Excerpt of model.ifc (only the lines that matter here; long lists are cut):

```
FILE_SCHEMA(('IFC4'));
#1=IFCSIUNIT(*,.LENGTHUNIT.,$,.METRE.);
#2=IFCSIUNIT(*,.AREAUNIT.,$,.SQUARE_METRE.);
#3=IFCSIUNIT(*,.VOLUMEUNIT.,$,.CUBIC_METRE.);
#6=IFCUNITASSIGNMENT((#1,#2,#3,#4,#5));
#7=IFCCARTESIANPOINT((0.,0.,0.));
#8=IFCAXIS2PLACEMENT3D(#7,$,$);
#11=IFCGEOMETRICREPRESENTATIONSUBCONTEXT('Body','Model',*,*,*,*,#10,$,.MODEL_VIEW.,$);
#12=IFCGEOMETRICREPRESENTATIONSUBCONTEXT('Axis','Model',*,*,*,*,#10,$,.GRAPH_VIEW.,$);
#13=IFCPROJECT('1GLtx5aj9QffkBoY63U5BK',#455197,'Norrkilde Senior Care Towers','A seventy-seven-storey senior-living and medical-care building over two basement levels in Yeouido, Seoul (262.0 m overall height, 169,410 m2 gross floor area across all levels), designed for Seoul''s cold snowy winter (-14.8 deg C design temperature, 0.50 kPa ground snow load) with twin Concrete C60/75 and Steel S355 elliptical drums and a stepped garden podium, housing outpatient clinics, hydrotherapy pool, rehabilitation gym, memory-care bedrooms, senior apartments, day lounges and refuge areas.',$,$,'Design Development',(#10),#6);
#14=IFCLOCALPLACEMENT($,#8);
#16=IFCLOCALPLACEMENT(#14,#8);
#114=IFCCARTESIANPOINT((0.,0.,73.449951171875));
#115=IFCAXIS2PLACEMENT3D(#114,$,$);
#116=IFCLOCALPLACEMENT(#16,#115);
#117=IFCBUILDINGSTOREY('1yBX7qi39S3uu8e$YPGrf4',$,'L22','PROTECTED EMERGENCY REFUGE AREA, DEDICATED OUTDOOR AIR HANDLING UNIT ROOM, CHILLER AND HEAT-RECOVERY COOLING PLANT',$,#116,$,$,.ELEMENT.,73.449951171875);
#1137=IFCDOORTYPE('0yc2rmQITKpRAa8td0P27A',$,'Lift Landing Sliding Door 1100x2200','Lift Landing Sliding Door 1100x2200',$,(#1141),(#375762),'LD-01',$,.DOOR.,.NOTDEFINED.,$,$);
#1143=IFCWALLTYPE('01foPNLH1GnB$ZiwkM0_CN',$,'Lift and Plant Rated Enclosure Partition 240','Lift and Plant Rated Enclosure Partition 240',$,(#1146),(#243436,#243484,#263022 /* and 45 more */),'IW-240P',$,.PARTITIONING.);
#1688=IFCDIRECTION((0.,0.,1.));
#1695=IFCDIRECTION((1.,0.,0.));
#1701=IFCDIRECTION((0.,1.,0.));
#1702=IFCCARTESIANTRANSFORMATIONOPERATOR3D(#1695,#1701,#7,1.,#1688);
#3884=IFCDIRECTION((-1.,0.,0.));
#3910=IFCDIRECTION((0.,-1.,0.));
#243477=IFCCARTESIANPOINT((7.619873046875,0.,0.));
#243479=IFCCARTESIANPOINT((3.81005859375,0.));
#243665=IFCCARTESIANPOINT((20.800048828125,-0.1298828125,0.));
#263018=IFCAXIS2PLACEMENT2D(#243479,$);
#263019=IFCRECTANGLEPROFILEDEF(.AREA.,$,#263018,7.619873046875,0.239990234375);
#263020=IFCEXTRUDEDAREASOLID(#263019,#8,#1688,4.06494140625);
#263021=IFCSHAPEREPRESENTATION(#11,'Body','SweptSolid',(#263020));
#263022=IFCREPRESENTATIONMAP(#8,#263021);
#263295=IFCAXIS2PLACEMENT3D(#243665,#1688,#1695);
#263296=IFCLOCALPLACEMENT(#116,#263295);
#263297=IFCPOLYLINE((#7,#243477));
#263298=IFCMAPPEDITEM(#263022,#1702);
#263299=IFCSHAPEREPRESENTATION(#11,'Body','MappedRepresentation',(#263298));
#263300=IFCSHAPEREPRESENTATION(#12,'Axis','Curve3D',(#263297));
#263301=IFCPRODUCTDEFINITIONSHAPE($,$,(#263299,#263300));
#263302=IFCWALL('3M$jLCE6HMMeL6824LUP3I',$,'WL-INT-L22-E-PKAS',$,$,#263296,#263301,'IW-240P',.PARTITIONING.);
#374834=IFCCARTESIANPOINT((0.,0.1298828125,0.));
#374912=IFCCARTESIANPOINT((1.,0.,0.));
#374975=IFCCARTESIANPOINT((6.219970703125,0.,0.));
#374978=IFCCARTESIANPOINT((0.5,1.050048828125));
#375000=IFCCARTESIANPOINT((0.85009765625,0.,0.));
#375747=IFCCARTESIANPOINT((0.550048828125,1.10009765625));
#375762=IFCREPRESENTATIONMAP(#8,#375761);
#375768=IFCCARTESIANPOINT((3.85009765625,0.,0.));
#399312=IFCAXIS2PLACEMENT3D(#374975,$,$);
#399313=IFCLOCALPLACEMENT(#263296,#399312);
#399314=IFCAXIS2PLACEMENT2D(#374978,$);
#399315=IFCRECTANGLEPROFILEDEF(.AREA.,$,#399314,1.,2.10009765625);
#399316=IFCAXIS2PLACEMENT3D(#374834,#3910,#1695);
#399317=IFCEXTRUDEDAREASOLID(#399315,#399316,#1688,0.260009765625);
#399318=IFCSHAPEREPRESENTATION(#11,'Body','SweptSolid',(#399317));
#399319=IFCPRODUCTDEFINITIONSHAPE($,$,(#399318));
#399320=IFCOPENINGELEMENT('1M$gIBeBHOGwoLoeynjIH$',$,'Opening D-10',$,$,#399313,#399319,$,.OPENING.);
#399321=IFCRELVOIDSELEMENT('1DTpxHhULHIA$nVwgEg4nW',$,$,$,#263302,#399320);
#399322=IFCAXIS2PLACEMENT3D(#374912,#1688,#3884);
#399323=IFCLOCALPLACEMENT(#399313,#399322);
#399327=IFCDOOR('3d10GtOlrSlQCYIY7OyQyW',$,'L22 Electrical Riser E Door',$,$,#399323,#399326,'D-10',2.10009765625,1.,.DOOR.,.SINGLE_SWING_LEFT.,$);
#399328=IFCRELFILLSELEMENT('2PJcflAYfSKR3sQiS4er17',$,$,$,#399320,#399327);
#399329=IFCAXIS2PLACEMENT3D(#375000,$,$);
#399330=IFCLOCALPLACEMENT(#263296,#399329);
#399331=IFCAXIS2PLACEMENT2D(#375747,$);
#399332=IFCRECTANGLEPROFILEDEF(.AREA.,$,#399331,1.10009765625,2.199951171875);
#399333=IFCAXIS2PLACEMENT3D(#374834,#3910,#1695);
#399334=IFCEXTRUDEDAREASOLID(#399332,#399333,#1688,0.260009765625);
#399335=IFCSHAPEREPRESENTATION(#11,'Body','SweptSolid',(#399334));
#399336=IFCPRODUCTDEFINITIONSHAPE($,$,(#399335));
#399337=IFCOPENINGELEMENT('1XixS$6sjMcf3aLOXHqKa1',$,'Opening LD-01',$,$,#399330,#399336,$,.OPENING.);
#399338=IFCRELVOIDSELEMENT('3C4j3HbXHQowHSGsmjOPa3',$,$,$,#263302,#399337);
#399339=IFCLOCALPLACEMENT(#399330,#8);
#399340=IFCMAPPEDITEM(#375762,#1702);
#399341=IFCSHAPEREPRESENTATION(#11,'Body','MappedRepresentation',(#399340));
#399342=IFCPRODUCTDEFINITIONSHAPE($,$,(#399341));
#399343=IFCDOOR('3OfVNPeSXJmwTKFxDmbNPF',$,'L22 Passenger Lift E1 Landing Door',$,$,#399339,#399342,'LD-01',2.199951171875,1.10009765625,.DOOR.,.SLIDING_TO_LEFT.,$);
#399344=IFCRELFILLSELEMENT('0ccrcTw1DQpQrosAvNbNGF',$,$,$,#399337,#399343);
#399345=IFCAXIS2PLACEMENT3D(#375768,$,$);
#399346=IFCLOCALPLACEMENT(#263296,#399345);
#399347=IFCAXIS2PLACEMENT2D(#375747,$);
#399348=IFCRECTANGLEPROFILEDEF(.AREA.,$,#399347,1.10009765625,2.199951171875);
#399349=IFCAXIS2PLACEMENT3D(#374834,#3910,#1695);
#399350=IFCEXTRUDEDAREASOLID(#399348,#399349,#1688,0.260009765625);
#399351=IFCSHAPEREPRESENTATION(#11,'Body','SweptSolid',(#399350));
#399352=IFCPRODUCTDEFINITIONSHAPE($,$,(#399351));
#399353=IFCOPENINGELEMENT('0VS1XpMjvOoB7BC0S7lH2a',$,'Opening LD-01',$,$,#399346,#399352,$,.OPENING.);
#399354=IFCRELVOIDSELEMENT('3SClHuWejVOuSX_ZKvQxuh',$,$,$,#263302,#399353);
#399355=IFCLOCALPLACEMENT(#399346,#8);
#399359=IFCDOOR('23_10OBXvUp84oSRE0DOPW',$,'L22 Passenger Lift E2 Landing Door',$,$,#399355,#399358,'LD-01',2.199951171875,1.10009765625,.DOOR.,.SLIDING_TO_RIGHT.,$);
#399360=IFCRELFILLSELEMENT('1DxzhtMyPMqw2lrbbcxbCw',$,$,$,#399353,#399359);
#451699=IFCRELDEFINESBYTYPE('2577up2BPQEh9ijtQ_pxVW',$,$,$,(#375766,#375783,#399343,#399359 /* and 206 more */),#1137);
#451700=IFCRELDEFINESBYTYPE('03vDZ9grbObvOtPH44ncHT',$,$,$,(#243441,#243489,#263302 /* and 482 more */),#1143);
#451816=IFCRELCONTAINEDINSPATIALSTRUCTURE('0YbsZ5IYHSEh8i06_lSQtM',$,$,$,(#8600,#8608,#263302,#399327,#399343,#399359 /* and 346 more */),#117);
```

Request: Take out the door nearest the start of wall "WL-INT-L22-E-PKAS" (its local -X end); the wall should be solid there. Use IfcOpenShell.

```python
import ifcopenshell
import ifcopenshell.api.feature
import ifcopenshell.api.root
import ifcopenshell.geom
import ifcopenshell.util.shape

model = ifcopenshell.open("model.ifc")
settings = ifcopenshell.geom.settings()


def volume(element):
    """Net volume in cubic metres, openings subtracted."""
    shape = ifcopenshell.geom.create_shape(settings, element)
    return ifcopenshell.util.shape.get_volume(shape.geometry)


door = model.by_id(399343)
opening = door.FillsVoids[0].RelatingOpeningElement
wall = opening.VoidsElements[0].RelatingBuildingElement
before = volume(wall)

ifcopenshell.api.root.remove_product(model, product=door)
ifcopenshell.api.feature.remove_feature(model, feature=opening)

after = volume(wall)

print(f"wall volume {before:.3f} -> {after:.3f} m3")

model.write("model-out.ifc")
```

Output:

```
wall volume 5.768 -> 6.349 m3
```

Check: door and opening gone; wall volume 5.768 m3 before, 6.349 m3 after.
